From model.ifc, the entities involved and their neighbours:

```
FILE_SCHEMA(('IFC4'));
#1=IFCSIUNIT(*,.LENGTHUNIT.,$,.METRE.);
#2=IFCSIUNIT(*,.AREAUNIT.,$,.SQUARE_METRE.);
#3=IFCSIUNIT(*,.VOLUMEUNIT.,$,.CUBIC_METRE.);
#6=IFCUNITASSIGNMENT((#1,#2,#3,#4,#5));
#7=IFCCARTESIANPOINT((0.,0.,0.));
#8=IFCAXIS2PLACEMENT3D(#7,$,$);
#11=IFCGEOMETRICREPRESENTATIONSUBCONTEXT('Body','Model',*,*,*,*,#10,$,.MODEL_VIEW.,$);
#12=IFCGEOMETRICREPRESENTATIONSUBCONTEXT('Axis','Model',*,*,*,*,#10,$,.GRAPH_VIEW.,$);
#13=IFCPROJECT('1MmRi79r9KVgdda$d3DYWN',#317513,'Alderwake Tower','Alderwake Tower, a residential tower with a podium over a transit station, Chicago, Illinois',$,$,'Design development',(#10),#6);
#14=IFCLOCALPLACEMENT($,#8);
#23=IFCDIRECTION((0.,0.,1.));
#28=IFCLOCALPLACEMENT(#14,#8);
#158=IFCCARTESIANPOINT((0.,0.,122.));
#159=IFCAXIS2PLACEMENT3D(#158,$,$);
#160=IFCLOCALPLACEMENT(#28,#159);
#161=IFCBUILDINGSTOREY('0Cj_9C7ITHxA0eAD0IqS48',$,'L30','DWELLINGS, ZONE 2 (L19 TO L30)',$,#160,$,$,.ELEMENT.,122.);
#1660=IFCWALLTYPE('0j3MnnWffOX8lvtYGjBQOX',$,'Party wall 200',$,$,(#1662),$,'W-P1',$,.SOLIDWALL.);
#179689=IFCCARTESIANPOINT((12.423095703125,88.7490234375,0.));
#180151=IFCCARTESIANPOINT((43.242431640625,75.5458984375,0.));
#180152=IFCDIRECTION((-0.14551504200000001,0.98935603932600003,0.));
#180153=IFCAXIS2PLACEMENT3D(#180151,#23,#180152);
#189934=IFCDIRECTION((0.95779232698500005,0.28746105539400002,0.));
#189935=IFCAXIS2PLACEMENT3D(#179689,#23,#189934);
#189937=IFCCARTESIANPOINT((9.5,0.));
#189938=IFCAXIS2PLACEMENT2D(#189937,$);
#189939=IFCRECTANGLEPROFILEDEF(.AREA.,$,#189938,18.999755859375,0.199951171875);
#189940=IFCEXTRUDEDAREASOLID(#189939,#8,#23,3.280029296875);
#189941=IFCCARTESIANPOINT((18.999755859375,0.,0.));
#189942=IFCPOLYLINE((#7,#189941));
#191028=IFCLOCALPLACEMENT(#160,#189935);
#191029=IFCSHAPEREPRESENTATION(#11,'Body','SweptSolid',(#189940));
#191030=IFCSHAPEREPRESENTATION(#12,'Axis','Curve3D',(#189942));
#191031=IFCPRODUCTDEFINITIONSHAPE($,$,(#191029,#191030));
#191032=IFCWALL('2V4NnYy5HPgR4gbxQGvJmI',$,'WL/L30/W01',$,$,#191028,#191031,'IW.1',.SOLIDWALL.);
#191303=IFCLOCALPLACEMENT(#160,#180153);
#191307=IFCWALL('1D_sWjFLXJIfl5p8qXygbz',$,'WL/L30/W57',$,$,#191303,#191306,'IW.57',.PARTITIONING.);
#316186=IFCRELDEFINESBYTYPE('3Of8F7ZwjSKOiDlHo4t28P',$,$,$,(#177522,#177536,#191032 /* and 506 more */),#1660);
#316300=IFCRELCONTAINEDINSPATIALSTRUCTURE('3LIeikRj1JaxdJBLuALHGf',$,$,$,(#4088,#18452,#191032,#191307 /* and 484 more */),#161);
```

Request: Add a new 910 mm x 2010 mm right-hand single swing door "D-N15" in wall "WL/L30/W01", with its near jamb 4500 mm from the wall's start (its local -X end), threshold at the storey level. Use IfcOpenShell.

```python
import numpy as np
import ifcopenshell
import ifcopenshell.api.feature
import ifcopenshell.api.geometry
import ifcopenshell.api.root
import ifcopenshell.api.spatial
import ifcopenshell.geom
import ifcopenshell.util.element
import ifcopenshell.util.placement
import ifcopenshell.util.representation
import ifcopenshell.util.shape
import ifcopenshell.util.unit

model = ifcopenshell.open("model.ifc")
unit_scale = ifcopenshell.util.unit.calculate_unit_scale(model)
settings = ifcopenshell.geom.settings()


def volume(element):
    """Net volume in cubic metres, openings subtracted."""
    shape = ifcopenshell.geom.create_shape(settings, element)
    return ifcopenshell.util.shape.get_volume(shape.geometry)


wall = model.by_guid("2V4NnYy5HPgR4gbxQGvJmI")
storey = ifcopenshell.util.element.get_container(wall, ifc_class="IfcBuildingStorey")
context = ifcopenshell.util.representation.get_context(model, "Model", "Body", "MODEL_VIEW")
before = volume(wall)

width, height, from_end, sill = 0.91, 2.01, 4.5, 0.0  # metres

# The wall runs along its own X axis, and the end named is its -X end.
wall_shape = ifcopenshell.geom.create_shape(settings, wall)
x, y, z = ifcopenshell.util.shape.get_vertices(wall_shape.geometry).T
start = x.min() + from_end
face, thickness = float(y.min()), float(y.max() - y.min())
wall_matrix = ifcopenshell.util.placement.get_local_placement(wall.ObjectPlacement)
level = ifcopenshell.util.placement.get_local_placement(storey.ObjectPlacement)[2, 3]


def in_wall(x, y):
    """Placement at x, y metres in the wall's axes, at sill height."""
    matrix = wall_matrix.copy()
    matrix[:, 3] = wall_matrix @ np.array([x / unit_scale, y / unit_scale, 0.0, 1.0])
    matrix[2, 3] = level + sill / unit_scale
    return matrix


# Opening: a box that overshoots both wall faces by 50 mm.
opening = ifcopenshell.api.root.create_entity(model, ifc_class="IfcOpeningElement", predefined_type="OPENING")
box = ifcopenshell.api.geometry.add_wall_representation(
    model, context=context, length=width, height=height, thickness=thickness + 0.1
)
ifcopenshell.api.geometry.assign_representation(model, product=opening, representation=box)
ifcopenshell.api.geometry.edit_object_placement(model, product=opening, matrix=in_wall(start, face - 0.05), is_si=False)
ifcopenshell.api.feature.add_feature(model, feature=opening, element=wall)

door = ifcopenshell.api.root.create_entity(model, ifc_class="IfcDoor", name="D-N15", predefined_type="DOOR")
door.OverallWidth, door.OverallHeight = width / unit_scale, height / unit_scale
door.OperationType = "SINGLE_SWING_RIGHT"
body = ifcopenshell.api.geometry.add_door_representation(
    model,
    context=context,
    overall_width=door.OverallWidth,
    overall_height=door.OverallHeight,
    operation_type="SINGLE_SWING_RIGHT",
    lining_properties={"LiningDepth": thickness / unit_scale, "ThresholdDepth": thickness / unit_scale},
)
ifcopenshell.api.geometry.assign_representation(model, product=door, representation=body)
ifcopenshell.api.spatial.assign_container(model, products=[door], relating_structure=storey)
ifcopenshell.api.feature.add_filling(model, opening=opening, element=door)

# The lining spans the wall, so the door starts at the wall face.
ifcopenshell.api.geometry.edit_object_placement(model, product=door, matrix=in_wall(start, face), is_si=False)

after = volume(wall)

print(f"wall volume {before:.3f} -> {after:.3f} m3")

model.write("model_v2.ifc")
```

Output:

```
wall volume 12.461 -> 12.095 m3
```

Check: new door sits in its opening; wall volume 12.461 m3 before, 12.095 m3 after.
